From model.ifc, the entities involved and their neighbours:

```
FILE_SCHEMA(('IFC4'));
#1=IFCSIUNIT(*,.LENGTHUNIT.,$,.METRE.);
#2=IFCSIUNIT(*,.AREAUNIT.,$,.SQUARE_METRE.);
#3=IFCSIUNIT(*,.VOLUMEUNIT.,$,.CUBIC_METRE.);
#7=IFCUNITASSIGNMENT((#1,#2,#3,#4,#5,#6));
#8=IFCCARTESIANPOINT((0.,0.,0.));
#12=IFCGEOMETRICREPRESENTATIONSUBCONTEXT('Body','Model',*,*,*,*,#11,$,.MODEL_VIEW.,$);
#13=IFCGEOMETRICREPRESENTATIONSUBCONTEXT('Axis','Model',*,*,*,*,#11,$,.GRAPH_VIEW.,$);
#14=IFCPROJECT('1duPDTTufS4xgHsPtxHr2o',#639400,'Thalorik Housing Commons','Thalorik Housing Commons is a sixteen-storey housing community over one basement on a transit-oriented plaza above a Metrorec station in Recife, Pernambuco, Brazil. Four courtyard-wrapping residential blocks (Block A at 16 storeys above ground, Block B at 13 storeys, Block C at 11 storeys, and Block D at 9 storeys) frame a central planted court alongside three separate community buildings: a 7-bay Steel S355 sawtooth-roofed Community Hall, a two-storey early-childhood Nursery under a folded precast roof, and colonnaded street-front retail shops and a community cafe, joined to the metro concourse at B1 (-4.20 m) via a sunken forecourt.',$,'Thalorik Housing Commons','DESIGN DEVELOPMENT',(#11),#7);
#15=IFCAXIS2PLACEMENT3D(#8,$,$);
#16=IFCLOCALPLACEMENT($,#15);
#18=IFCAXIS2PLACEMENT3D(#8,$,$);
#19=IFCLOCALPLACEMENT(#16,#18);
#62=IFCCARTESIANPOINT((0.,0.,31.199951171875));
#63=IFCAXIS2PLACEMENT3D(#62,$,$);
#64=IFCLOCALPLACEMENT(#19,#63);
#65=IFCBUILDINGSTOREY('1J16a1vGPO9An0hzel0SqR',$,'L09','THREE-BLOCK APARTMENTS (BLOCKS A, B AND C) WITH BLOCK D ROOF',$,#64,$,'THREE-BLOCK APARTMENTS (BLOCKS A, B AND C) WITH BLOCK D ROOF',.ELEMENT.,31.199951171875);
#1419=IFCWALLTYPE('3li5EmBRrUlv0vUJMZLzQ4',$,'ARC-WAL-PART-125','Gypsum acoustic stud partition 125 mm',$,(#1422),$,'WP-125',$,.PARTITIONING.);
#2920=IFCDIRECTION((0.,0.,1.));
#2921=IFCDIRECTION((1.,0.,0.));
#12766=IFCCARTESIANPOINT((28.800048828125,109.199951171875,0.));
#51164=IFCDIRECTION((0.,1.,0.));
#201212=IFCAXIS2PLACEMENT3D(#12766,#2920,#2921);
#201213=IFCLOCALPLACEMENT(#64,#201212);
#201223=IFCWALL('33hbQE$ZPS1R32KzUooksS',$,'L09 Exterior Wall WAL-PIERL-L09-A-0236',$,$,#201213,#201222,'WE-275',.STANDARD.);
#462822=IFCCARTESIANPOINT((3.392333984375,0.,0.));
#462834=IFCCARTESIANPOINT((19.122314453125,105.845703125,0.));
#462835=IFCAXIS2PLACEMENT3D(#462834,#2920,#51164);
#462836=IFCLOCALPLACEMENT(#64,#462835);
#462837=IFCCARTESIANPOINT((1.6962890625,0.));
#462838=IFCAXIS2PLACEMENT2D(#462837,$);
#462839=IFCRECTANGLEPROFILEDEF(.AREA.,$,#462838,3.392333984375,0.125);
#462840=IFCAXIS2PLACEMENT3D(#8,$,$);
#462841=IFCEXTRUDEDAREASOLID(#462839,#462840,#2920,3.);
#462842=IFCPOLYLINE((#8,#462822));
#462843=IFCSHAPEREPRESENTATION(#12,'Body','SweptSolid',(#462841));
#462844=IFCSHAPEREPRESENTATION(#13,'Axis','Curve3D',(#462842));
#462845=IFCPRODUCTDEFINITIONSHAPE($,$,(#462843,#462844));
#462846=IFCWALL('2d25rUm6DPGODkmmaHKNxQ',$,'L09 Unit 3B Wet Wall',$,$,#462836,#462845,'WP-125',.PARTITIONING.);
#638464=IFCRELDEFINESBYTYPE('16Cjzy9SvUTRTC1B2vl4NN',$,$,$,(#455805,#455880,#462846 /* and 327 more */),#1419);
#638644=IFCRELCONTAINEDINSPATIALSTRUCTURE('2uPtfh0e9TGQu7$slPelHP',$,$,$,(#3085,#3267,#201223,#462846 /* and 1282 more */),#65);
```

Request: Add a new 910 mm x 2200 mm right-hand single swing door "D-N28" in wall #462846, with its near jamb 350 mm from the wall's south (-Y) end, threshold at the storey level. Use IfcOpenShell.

```python
import numpy as np
import ifcopenshell
import ifcopenshell.api.feature
import ifcopenshell.api.geometry
import ifcopenshell.api.root
import ifcopenshell.api.spatial
import ifcopenshell.geom
import ifcopenshell.util.element
import ifcopenshell.util.placement
import ifcopenshell.util.representation
import ifcopenshell.util.shape
import ifcopenshell.util.unit

model = ifcopenshell.open("model.ifc")
unit_scale = ifcopenshell.util.unit.calculate_unit_scale(model)
settings = ifcopenshell.geom.settings()


def volume(element):
    """Net volume in cubic metres, openings subtracted."""
    shape = ifcopenshell.geom.create_shape(settings, element)
    return ifcopenshell.util.shape.get_volume(shape.geometry)


wall = model.by_guid("2d25rUm6DPGODkmmaHKNxQ")
storey = ifcopenshell.util.element.get_container(wall, ifc_class="IfcBuildingStorey")
context = ifcopenshell.util.representation.get_context(model, "Model", "Body", "MODEL_VIEW")
before = volume(wall)

width, height, from_end, sill = 0.91, 2.2, 0.35, 0.0  # metres

# The wall runs along its own X axis, and the end named is its -X end.
wall_shape = ifcopenshell.geom.create_shape(settings, wall)
x, y, z = ifcopenshell.util.shape.get_vertices(wall_shape.geometry).T
start = x.min() + from_end
face, thickness = float(y.min()), float(y.max() - y.min())
wall_matrix = ifcopenshell.util.placement.get_local_placement(wall.ObjectPlacement)
level = ifcopenshell.util.placement.get_local_placement(storey.ObjectPlacement)[2, 3]


def in_wall(x, y):
    """Placement at x, y metres in the wall's axes, at sill height."""
    matrix = wall_matrix.copy()
    matrix[:, 3] = wall_matrix @ np.array([x / unit_scale, y / unit_scale, 0.0, 1.0])
    matrix[2, 3] = level + sill / unit_scale
    return matrix


# Opening: a box that overshoots both wall faces by 50 mm.
opening = ifcopenshell.api.root.create_entity(model, ifc_class="IfcOpeningElement", predefined_type="OPENING")
box = ifcopenshell.api.geometry.add_wall_representation(
    model, context=context, length=width, height=height, thickness=thickness + 0.1
)
ifcopenshell.api.geometry.assign_representation(model, product=opening, representation=box)
ifcopenshell.api.geometry.edit_object_placement(model, product=opening, matrix=in_wall(start, face - 0.05), is_si=False)
ifcopenshell.api.feature.add_feature(model, feature=opening, element=wall)

door = ifcopenshell.api.root.create_entity(model, ifc_class="IfcDoor", name="D-N28", predefined_type="DOOR")
door.OverallWidth, door.OverallHeight = width / unit_scale, height / unit_scale
door.OperationType = "SINGLE_SWING_RIGHT"
body = ifcopenshell.api.geometry.add_door_representation(
    model,
    context=context,
    overall_width=door.OverallWidth,
    overall_height=door.OverallHeight,
    operation_type="SINGLE_SWING_RIGHT",
    lining_properties={"LiningDepth": thickness / unit_scale, "ThresholdDepth": thickness / unit_scale},
)
ifcopenshell.api.geometry.assign_representation(model, product=door, representation=body)
ifcopenshell.api.spatial.assign_container(model, products=[door], relating_structure=storey)
ifcopenshell.api.feature.add_filling(model, opening=opening, element=door)

# The lining spans the wall, so the door starts at the wall face.
ifcopenshell.api.geometry.edit_object_placement(model, product=door, matrix=in_wall(start, face), is_si=False)

after = volume(wall)

print(f"wall volume {before:.3f} -> {after:.3f} m3")

model.write("model_rev.ifc")
```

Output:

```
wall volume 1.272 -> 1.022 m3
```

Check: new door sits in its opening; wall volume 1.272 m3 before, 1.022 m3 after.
